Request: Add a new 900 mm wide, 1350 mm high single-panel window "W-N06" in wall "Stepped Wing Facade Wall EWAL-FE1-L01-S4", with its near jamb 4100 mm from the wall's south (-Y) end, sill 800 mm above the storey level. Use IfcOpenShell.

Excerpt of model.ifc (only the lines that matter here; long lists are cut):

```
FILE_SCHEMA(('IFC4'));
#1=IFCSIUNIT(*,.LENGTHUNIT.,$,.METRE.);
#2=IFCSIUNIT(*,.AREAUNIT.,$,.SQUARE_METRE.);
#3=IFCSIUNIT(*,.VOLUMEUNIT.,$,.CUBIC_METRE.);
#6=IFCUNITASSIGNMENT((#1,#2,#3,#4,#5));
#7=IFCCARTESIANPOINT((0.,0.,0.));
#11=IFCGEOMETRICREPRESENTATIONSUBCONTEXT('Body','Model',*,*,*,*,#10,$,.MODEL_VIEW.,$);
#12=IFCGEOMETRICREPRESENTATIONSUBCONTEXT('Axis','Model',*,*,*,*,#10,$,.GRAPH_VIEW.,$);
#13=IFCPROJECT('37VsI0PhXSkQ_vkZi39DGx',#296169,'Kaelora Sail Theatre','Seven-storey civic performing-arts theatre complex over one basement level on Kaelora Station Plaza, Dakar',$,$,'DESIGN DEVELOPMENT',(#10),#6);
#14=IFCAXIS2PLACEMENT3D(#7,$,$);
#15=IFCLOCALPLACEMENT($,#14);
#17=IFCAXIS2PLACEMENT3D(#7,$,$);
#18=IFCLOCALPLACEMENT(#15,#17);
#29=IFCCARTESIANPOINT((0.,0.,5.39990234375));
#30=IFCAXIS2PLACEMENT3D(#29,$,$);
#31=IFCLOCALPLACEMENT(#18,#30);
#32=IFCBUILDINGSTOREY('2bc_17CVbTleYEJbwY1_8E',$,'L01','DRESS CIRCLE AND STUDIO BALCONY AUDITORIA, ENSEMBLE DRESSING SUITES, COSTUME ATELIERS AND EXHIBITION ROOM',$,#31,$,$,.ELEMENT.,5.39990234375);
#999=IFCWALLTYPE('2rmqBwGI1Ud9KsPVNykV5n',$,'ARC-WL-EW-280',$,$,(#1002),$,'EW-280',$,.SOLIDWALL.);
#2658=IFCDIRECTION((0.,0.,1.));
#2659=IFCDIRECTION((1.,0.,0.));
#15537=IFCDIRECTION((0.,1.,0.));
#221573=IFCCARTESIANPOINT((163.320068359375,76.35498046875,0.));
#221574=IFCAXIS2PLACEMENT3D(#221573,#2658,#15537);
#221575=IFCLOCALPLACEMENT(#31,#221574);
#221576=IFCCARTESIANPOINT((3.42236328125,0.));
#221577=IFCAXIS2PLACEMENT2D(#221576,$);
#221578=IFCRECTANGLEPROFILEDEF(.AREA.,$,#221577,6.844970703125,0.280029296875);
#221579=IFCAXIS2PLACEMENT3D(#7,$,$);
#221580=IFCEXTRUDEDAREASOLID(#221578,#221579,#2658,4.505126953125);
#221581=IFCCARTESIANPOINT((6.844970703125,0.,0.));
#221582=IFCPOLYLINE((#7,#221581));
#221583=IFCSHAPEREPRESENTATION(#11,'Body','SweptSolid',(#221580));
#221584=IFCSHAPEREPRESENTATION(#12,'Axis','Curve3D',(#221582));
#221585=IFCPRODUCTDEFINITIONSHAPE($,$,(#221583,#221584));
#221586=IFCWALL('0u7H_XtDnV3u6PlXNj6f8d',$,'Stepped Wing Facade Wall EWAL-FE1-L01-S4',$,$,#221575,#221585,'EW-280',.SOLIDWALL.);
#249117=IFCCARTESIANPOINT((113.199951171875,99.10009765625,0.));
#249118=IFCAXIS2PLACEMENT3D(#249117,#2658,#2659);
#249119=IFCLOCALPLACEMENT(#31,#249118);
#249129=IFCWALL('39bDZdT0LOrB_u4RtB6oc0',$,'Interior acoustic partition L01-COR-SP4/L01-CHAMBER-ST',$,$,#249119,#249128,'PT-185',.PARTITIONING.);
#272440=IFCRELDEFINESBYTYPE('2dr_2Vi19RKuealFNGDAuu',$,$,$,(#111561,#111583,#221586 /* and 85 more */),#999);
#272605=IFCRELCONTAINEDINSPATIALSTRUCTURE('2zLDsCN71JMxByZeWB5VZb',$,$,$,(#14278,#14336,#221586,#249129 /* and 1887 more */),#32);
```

```python
import numpy as np
import ifcopenshell
import ifcopenshell.api.feature
import ifcopenshell.api.geometry
import ifcopenshell.api.root
import ifcopenshell.api.spatial
import ifcopenshell.geom
import ifcopenshell.util.element
import ifcopenshell.util.placement
import ifcopenshell.util.representation
import ifcopenshell.util.shape
import ifcopenshell.util.unit

model = ifcopenshell.open("model.ifc")
unit_scale = ifcopenshell.util.unit.calculate_unit_scale(model)
settings = ifcopenshell.geom.settings()


def volume(element):
    """Net volume in cubic metres, openings subtracted."""
    shape = ifcopenshell.geom.create_shape(settings, element)
    return ifcopenshell.util.shape.get_volume(shape.geometry)


wall = model.by_guid("0u7H_XtDnV3u6PlXNj6f8d")
storey = ifcopenshell.util.element.get_container(wall, ifc_class="IfcBuildingStorey")
context = ifcopenshell.util.representation.get_context(model, "Model", "Body", "MODEL_VIEW")
before = volume(wall)

width, height, from_end, sill = 0.9, 1.35, 4.1, 0.8  # metres

# The wall runs along its own X axis, and the end named is its -X end.
wall_shape = ifcopenshell.geom.create_shape(settings, wall)
x, y, z = ifcopenshell.util.shape.get_vertices(wall_shape.geometry).T
start = x.min() + from_end
face, thickness = float(y.min()), float(y.max() - y.min())
wall_matrix = ifcopenshell.util.placement.get_local_placement(wall.ObjectPlacement)
level = ifcopenshell.util.placement.get_local_placement(storey.ObjectPlacement)[2, 3]


def in_wall(x, y):
    """Placement at x, y metres in the wall's axes, at sill height."""
    matrix = wall_matrix.copy()
    matrix[:, 3] = wall_matrix @ np.array([x / unit_scale, y / unit_scale, 0.0, 1.0])
    matrix[2, 3] = level + sill / unit_scale
    return matrix


# Opening: a box that overshoots both wall faces by 50 mm.
opening = ifcopenshell.api.root.create_entity(model, ifc_class="IfcOpeningElement", predefined_type="OPENING")
box = ifcopenshell.api.geometry.add_wall_representation(
    model, context=context, length=width, height=height, thickness=thickness + 0.1
)
ifcopenshell.api.geometry.assign_representation(model, product=opening, representation=box)
ifcopenshell.api.geometry.edit_object_placement(model, product=opening, matrix=in_wall(start, face - 0.05), is_si=False)
ifcopenshell.api.feature.add_feature(model, feature=opening, element=wall)

window = ifcopenshell.api.root.create_entity(model, ifc_class="IfcWindow", name="W-N06", predefined_type="WINDOW")
window.OverallWidth, window.OverallHeight = width / unit_scale, height / unit_scale
window.PartitioningType = "SINGLE_PANEL"
body = ifcopenshell.api.geometry.add_window_representation(
    model,
    context=context,
    overall_width=window.OverallWidth,
    overall_height=window.OverallHeight,
    partition_type="SINGLE_PANEL",
)
ifcopenshell.api.geometry.assign_representation(model, product=window, representation=body)
ifcopenshell.api.spatial.assign_container(model, products=[window], relating_structure=storey)
ifcopenshell.api.feature.add_filling(model, opening=opening, element=window)

# Centre the window in the wall's thickness.
ifcopenshell.api.geometry.edit_object_placement(model, product=window, matrix=in_wall(start, face), is_si=False)
window_shape = ifcopenshell.geom.create_shape(settings, window)
depth = ifcopenshell.util.shape.get_vertices(window_shape.geometry)[:, 1]
offset = face + thickness / 2 - (depth.min() + depth.max()) / 2
ifcopenshell.api.geometry.edit_object_placement(model, product=window, matrix=in_wall(start, offset), is_si=False)

after = volume(wall)

print(f"wall volume {before:.3f} -> {after:.3f} m3")

model.write("model_updated.ifc")
```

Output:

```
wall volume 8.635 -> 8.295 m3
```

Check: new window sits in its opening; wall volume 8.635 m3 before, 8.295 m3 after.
